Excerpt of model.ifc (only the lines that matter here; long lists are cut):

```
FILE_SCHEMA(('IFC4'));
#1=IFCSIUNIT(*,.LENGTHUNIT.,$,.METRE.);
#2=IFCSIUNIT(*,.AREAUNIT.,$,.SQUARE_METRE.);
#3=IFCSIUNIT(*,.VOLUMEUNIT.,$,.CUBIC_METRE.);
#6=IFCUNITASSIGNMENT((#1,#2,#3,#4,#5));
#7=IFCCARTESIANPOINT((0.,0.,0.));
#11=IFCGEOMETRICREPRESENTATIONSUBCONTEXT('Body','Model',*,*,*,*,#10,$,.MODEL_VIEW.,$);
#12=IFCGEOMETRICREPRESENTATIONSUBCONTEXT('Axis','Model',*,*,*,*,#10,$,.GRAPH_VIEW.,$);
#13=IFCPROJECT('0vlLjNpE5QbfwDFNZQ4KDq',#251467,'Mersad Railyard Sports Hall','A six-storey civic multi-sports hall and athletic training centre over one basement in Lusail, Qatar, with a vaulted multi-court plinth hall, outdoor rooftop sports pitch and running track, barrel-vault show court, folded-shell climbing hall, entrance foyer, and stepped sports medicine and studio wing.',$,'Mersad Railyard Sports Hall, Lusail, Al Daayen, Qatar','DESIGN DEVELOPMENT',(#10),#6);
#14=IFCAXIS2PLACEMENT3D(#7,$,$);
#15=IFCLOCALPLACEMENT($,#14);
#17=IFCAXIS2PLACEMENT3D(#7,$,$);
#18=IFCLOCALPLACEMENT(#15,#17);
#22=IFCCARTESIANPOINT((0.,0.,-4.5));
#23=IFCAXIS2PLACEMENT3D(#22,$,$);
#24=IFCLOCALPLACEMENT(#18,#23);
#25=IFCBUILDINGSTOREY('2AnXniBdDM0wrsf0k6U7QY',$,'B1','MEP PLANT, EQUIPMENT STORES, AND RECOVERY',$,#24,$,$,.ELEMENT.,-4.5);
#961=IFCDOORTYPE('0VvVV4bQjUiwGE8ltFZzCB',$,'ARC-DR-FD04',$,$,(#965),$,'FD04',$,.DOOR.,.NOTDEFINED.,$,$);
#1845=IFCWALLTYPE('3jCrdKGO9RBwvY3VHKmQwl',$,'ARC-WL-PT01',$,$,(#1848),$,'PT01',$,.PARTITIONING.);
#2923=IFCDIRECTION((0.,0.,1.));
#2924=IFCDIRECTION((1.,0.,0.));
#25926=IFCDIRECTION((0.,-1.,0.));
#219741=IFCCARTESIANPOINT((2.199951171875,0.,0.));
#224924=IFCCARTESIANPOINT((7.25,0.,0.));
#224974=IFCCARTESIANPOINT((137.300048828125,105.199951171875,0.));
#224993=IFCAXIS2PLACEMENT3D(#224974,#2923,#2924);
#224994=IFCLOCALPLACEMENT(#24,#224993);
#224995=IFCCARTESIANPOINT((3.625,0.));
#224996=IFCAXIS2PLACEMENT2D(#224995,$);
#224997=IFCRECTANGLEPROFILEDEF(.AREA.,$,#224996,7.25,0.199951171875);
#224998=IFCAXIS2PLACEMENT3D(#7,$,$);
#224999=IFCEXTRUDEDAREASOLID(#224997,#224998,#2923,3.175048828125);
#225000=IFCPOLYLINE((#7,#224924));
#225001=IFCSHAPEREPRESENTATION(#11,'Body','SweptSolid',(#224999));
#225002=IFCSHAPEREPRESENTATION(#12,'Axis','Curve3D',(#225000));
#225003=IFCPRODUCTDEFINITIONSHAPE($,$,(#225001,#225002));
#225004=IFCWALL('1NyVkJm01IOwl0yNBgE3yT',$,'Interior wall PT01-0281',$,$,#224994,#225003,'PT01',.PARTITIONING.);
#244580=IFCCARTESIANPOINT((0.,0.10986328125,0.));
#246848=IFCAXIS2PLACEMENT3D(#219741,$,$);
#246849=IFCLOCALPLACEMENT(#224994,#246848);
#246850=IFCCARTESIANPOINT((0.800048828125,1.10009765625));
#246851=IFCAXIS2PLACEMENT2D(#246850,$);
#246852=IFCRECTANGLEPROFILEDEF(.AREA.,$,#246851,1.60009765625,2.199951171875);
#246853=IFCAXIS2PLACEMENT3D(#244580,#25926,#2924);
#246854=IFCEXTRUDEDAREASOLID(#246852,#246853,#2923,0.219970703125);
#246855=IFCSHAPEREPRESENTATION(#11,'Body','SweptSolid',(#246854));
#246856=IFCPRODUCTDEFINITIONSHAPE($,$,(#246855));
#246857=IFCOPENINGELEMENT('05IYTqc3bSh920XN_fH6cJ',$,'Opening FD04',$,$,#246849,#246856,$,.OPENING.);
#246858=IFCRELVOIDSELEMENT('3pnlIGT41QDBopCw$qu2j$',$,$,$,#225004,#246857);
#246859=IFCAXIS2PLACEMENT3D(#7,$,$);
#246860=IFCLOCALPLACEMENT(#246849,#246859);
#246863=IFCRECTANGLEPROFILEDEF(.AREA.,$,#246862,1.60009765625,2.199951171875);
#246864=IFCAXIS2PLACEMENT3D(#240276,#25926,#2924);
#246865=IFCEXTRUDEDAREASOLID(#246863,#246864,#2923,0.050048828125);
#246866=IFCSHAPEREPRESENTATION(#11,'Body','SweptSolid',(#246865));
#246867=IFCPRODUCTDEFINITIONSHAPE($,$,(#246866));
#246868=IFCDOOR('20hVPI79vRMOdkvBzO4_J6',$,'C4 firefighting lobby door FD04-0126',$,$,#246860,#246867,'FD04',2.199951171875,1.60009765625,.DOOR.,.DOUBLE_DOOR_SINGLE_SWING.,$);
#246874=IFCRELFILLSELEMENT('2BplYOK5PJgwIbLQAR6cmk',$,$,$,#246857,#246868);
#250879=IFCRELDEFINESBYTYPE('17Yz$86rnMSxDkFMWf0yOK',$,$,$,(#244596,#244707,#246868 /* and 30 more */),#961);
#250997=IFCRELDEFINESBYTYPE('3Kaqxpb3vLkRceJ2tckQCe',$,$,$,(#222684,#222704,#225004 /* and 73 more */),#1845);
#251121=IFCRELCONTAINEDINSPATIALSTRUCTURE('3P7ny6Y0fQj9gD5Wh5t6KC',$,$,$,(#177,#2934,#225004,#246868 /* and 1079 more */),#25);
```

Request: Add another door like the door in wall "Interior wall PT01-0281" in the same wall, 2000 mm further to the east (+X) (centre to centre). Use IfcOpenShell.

```python
import ifcopenshell
import ifcopenshell.api.feature
import ifcopenshell.api.geometry
import ifcopenshell.api.root
import ifcopenshell.geom
import ifcopenshell.util.element
import ifcopenshell.util.placement
import ifcopenshell.util.shape
import ifcopenshell.util.unit

model = ifcopenshell.open("model.ifc")
unit_scale = ifcopenshell.util.unit.calculate_unit_scale(model)
settings = ifcopenshell.geom.settings()


def volume(element):
    """Net volume in cubic metres, openings subtracted."""
    shape = ifcopenshell.geom.create_shape(settings, element)
    return ifcopenshell.util.shape.get_volume(shape.geometry)


door = model.by_guid("20hVPI79vRMOdkvBzO4_J6")
opening = door.FillsVoids[0].RelatingOpeningElement
wall = opening.VoidsElements[0].RelatingBuildingElement
before = volume(wall)
shift = ifcopenshell.util.placement.get_local_placement(wall.ObjectPlacement)[:3, 0] * 2 / unit_scale

# copy_class copies the void relationship, type, container and properties, but no geometry.
new_opening = ifcopenshell.api.root.copy_class(model, product=opening)
new_opening.Representation = ifcopenshell.util.element.copy_deep(
    model, opening.Representation, exclude=["IfcGeometricRepresentationContext", "IfcRepresentationMap"]
)
new_door = ifcopenshell.api.root.copy_class(model, product=door)
new_door.Representation = ifcopenshell.util.element.copy_deep(
    model, door.Representation, exclude=["IfcGeometricRepresentationContext", "IfcRepresentationMap"]
)
new_door.Tag = None
ifcopenshell.api.feature.add_filling(model, opening=new_opening, element=new_door)

for old, new in ((opening, new_opening), (door, new_door)):
    matrix = ifcopenshell.util.placement.get_local_placement(old.ObjectPlacement)
    matrix[:3, 3] += shift
    ifcopenshell.api.geometry.edit_object_placement(model, product=new, matrix=matrix, is_si=False)

after = volume(wall)

print(f"wall volume {before:.3f} -> {after:.3f} m3")

model.write("model-out.ifc")
```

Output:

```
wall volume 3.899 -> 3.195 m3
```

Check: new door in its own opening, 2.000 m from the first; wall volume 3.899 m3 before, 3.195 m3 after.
